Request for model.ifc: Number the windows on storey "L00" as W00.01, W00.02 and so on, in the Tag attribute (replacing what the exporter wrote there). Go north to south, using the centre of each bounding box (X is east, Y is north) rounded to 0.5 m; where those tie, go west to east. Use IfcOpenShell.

First a look at what the model holds.

```python
import ifcopenshell
import ifcopenshell.util.element
import ifcopenshell.util.placement

model = ifcopenshell.open("model.ifc")
print(model.schema)
storey = next(s for s in model.by_type("IfcBuildingStorey") if s.Name == "L00")
windows = [e for e in ifcopenshell.util.element.get_decomposition(storey) if e.is_a("IfcWindow")]
for e in sorted(windows, key=lambda e: e.id()):
    origin = ifcopenshell.util.placement.get_local_placement(e.ObjectPlacement)[:3, 3]
    print(e.id(), e.Tag, e.Name, origin.round(2) + 0.0, sep=" | ")
```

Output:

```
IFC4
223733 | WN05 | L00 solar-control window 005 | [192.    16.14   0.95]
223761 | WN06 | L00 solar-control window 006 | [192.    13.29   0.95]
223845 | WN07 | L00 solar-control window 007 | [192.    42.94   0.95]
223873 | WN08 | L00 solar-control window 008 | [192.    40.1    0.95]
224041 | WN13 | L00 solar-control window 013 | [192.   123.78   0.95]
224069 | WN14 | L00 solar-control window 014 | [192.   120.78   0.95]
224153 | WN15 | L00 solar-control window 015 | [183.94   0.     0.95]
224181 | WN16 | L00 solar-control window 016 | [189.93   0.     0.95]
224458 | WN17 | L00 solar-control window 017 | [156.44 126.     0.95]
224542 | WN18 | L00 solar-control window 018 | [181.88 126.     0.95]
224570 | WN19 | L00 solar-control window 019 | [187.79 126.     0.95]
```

```python
import ifcopenshell
import ifcopenshell.geom
import ifcopenshell.util.element
import ifcopenshell.util.shape

model = ifcopenshell.open("model.ifc")
settings = ifcopenshell.geom.settings()
settings.set("use-world-coords", True)


def centre(element):
    shape = ifcopenshell.geom.create_shape(settings, element)
    return ifcopenshell.util.shape.get_bbox_centroid(shape.geometry)


storey = next(s for s in model.by_type("IfcBuildingStorey") if s.Name == "L00")
windows = [e for e in ifcopenshell.util.element.get_decomposition(storey) if e.is_a("IfcWindow")]

# Insertion points can sit at a corner or the storey origin, so sort by the geometry (in metres).
centres = {e: centre(e) for e in windows}
windows.sort(key=lambda e: (-round(centres[e][1] / 0.5), centres[e][0]))

for i, e in enumerate(windows, start=1):
    number = f"W00.{i:02d}"
    e.Tag = number
    print(e.id(), number)

model.write("model_updated.ifc")
```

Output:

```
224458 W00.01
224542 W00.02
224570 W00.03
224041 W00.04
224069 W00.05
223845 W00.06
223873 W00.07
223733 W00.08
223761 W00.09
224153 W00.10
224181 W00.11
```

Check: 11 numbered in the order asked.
